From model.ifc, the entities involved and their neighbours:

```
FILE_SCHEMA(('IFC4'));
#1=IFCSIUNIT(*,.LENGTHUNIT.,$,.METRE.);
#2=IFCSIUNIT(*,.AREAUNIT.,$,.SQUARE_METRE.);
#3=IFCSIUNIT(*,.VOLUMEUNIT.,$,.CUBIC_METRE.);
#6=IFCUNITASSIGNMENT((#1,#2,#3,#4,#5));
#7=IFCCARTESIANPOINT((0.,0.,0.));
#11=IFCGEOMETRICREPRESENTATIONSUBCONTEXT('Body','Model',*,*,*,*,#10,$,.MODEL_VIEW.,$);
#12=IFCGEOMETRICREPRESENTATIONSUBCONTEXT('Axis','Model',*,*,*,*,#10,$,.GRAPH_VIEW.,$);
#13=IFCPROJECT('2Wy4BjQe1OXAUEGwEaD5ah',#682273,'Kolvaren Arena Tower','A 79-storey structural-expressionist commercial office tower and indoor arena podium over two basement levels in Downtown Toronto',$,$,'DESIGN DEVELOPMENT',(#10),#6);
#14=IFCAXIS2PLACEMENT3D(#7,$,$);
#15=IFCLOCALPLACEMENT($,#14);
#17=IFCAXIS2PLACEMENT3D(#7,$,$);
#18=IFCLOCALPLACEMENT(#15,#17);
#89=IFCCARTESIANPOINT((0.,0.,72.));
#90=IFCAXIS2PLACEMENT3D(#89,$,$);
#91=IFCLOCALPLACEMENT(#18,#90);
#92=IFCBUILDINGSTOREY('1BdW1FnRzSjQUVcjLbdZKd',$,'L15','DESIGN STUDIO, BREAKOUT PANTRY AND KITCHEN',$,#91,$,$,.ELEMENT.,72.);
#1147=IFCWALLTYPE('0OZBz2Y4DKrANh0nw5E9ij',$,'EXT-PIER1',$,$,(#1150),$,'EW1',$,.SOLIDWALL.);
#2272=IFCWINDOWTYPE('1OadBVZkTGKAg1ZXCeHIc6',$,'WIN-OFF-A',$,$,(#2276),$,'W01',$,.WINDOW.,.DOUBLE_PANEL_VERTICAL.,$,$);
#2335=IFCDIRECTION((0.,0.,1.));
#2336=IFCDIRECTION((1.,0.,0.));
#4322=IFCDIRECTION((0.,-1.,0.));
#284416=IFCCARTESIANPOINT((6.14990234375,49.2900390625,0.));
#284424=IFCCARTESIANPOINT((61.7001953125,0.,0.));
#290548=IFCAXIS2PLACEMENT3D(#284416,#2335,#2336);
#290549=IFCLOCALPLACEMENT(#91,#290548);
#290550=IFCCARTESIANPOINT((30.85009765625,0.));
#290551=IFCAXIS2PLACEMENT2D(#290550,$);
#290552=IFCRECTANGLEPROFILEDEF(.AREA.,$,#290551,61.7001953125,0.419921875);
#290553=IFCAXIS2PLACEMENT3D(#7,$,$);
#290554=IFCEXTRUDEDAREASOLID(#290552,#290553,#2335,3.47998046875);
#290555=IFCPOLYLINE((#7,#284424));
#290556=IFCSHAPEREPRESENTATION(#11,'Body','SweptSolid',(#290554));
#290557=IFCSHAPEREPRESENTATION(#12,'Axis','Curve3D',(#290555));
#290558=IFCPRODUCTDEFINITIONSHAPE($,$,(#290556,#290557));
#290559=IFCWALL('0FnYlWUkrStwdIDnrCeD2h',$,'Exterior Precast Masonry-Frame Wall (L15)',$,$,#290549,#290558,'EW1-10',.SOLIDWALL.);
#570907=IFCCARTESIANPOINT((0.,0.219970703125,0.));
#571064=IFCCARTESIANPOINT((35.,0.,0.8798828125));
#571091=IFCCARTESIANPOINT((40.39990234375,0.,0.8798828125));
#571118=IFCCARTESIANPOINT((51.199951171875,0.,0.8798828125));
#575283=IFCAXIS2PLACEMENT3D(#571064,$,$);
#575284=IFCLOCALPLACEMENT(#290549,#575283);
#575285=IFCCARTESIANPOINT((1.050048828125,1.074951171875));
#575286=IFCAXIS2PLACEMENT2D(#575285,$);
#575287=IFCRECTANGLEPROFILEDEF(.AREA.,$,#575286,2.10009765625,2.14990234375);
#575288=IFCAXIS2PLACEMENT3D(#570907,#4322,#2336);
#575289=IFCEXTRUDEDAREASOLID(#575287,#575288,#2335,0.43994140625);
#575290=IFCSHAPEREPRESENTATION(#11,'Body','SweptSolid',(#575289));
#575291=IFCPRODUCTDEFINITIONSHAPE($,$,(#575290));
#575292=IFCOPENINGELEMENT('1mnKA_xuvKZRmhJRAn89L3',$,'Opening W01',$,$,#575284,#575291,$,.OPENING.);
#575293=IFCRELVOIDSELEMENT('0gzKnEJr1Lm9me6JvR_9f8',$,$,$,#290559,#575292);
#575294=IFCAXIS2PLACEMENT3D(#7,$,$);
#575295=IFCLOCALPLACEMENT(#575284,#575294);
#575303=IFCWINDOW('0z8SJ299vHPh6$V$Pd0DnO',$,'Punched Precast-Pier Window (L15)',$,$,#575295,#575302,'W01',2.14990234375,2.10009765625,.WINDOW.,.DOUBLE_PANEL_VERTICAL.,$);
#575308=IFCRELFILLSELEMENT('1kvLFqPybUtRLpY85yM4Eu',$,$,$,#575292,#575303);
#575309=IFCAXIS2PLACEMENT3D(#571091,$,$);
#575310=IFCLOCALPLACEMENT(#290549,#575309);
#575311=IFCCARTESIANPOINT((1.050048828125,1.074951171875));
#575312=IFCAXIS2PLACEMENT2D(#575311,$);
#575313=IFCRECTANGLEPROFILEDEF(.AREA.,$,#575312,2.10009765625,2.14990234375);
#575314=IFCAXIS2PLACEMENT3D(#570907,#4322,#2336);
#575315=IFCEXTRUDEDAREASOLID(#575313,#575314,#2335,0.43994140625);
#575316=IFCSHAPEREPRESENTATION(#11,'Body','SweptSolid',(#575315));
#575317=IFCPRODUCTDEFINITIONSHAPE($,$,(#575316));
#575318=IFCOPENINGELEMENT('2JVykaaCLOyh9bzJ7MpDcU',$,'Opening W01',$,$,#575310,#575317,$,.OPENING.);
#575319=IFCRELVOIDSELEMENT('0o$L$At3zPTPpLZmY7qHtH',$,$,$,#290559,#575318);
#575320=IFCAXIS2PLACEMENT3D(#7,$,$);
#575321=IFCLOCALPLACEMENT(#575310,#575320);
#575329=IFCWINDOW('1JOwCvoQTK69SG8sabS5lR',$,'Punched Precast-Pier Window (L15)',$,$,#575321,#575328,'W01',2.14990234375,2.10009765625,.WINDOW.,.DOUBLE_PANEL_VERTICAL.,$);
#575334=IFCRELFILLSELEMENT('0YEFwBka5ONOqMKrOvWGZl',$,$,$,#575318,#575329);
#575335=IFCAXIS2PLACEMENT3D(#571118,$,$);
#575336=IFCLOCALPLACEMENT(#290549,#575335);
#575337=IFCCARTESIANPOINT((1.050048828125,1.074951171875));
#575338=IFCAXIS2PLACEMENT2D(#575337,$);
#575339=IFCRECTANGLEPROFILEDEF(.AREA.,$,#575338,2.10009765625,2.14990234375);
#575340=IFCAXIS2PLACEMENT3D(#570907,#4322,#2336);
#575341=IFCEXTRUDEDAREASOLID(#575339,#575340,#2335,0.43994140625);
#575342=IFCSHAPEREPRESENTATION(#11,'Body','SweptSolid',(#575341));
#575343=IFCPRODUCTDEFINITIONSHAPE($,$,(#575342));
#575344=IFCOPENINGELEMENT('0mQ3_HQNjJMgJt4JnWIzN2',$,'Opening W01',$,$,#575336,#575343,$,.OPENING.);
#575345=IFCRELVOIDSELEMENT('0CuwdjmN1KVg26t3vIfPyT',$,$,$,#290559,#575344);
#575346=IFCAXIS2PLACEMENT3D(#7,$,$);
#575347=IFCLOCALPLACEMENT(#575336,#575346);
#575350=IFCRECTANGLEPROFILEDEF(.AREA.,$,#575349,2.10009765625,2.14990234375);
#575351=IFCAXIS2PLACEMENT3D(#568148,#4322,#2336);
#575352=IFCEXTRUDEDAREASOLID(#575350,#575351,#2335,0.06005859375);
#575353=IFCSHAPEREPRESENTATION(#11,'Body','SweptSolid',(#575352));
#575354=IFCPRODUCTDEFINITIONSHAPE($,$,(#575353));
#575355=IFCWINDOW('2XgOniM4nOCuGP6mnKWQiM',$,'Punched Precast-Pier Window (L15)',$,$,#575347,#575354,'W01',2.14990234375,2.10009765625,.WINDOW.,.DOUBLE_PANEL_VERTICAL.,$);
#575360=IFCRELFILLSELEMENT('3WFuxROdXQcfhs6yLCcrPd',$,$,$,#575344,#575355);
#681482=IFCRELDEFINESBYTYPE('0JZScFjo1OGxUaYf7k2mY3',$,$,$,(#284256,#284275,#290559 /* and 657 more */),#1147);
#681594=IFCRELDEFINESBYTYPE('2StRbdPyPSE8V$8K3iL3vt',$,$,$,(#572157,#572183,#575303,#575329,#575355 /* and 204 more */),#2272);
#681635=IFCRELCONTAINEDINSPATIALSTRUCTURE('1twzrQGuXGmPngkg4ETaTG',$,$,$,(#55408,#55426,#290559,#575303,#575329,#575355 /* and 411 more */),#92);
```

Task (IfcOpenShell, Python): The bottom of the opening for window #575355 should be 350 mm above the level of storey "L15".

```python
import numpy as np
import ifcopenshell
import ifcopenshell.api.geometry
import ifcopenshell.geom
import ifcopenshell.util.element
import ifcopenshell.util.placement
import ifcopenshell.util.shape
import ifcopenshell.util.unit

model = ifcopenshell.open("model.ifc")
unit_scale = ifcopenshell.util.unit.calculate_unit_scale(model)

window = model.by_id(575355)
opening = window.FillsVoids[0].RelatingOpeningElement
storey = ifcopenshell.util.element.get_container(window, ifc_class="IfcBuildingStorey")
level = ifcopenshell.util.placement.get_local_placement(storey.ObjectPlacement)[2, 3]

# The opening's origin need not be at the sill, so measure its lowest point.
shape = ifcopenshell.geom.create_shape(ifcopenshell.geom.settings(), opening)
bottom = ifcopenshell.util.shape.get_shape_bottom_elevation(shape, shape.geometry) / unit_scale
dz = level + 0.35 / unit_scale - bottom

shift = np.array([0.0, 0.0, dz])
# The window is placed relative to its opening, so it follows when the opening moves.
matrix = ifcopenshell.util.placement.get_local_placement(opening.ObjectPlacement)
matrix[:3, 3] += shift
ifcopenshell.api.geometry.edit_object_placement(
    model, product=opening, matrix=matrix, is_si=False, should_transform_children=True
)

print(f"moved by {dz * unit_scale:+.3f} m")

model.write("model_updated.ifc")
```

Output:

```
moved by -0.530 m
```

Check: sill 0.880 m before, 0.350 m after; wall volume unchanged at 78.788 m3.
